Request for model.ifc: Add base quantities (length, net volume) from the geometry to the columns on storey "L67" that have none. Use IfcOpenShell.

First a look at what the model holds.

```python
import ifcopenshell
import ifcopenshell.util.element
import ifcopenshell.util.unit

model = ifcopenshell.open("model.ifc")
print(model.schema)
for unit_type in ("LENGTHUNIT", "AREAUNIT", "VOLUMEUNIT"):
    print(unit_type, ifcopenshell.util.unit.calculate_unit_scale(model, unit_type))
storey = next(s for s in model.by_type("IfcBuildingStorey") if s.Name == "L67")
columns = [e for e in ifcopenshell.util.element.get_decomposition(storey) if e.is_a("IfcColumn")]
for e in sorted(columns, key=lambda e: e.id()):
    print(e.id(), e.is_a(), e.Name, list(ifcopenshell.util.element.get_psets(e, qtos_only=True)), sep=" | ")
```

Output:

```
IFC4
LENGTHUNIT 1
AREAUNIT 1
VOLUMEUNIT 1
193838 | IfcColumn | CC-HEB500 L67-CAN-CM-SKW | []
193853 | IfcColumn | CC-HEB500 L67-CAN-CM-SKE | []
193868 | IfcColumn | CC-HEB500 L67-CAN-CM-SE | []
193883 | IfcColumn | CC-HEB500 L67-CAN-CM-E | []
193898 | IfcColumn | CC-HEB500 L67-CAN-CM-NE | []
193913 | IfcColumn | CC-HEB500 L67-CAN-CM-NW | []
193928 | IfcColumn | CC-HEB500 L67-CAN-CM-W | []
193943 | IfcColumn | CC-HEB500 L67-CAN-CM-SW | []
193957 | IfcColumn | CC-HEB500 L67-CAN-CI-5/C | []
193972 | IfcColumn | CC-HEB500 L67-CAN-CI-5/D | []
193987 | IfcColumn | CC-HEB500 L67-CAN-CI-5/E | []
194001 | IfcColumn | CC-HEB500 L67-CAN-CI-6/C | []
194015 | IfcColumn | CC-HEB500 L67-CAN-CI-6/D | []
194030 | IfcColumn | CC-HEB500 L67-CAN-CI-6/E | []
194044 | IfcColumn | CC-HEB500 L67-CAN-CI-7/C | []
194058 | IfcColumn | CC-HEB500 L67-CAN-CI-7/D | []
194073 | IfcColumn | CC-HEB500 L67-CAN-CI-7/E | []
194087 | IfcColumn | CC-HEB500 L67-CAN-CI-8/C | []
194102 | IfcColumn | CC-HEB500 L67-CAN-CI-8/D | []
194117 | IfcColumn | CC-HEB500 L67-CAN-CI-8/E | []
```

```python
import ifcopenshell
import ifcopenshell.api.pset
import ifcopenshell.geom
import ifcopenshell.util.element
import ifcopenshell.util.shape
import ifcopenshell.util.unit

model = ifcopenshell.open("model.ifc")
unit_scale = ifcopenshell.util.unit.calculate_unit_scale(model)
volume_scale = ifcopenshell.util.unit.calculate_unit_scale(model, "VOLUMEUNIT")
settings = ifcopenshell.geom.settings()

storey = next(s for s in model.by_type("IfcBuildingStorey") if s.Name == "L67")
columns = [e for e in ifcopenshell.util.element.get_decomposition(storey) if e.is_a("IfcColumn")]

for e in sorted(columns, key=lambda e: e.id()):
    if ifcopenshell.util.element.get_psets(e, qtos_only=True, should_inherit=False):
        continue
    # Geometry comes back in metres, in the element's own axes.
    shape = ifcopenshell.geom.create_shape(settings, e)
    values = {
        "Length": ifcopenshell.util.shape.get_z(shape.geometry) / unit_scale,
        "NetVolume": ifcopenshell.util.shape.get_volume(shape.geometry) / volume_scale,
    }
    qto = ifcopenshell.api.pset.add_qto(model, product=e, name="Qto_ColumnBaseQuantities")
    ifcopenshell.api.pset.edit_qto(model, qto=qto, properties=values)
    print(e.id(), {k: round(v, 3) for k, v in values.items()})

model.write("model_rev.ifc")
```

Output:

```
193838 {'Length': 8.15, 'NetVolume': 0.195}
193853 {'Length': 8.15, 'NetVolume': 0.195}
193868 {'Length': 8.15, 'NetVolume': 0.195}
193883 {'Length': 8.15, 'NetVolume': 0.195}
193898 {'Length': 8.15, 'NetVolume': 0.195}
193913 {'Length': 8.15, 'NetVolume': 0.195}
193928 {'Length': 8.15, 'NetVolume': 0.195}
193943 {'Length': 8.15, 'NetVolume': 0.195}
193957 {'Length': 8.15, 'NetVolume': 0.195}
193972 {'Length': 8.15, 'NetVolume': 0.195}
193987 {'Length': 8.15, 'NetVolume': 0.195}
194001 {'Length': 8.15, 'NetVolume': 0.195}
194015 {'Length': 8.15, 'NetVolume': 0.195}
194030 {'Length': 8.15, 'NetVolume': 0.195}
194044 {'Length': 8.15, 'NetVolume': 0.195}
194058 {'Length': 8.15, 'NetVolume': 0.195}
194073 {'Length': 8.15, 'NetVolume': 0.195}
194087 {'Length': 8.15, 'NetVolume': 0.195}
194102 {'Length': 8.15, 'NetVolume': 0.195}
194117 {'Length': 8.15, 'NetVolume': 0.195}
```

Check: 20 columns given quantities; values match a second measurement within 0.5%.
